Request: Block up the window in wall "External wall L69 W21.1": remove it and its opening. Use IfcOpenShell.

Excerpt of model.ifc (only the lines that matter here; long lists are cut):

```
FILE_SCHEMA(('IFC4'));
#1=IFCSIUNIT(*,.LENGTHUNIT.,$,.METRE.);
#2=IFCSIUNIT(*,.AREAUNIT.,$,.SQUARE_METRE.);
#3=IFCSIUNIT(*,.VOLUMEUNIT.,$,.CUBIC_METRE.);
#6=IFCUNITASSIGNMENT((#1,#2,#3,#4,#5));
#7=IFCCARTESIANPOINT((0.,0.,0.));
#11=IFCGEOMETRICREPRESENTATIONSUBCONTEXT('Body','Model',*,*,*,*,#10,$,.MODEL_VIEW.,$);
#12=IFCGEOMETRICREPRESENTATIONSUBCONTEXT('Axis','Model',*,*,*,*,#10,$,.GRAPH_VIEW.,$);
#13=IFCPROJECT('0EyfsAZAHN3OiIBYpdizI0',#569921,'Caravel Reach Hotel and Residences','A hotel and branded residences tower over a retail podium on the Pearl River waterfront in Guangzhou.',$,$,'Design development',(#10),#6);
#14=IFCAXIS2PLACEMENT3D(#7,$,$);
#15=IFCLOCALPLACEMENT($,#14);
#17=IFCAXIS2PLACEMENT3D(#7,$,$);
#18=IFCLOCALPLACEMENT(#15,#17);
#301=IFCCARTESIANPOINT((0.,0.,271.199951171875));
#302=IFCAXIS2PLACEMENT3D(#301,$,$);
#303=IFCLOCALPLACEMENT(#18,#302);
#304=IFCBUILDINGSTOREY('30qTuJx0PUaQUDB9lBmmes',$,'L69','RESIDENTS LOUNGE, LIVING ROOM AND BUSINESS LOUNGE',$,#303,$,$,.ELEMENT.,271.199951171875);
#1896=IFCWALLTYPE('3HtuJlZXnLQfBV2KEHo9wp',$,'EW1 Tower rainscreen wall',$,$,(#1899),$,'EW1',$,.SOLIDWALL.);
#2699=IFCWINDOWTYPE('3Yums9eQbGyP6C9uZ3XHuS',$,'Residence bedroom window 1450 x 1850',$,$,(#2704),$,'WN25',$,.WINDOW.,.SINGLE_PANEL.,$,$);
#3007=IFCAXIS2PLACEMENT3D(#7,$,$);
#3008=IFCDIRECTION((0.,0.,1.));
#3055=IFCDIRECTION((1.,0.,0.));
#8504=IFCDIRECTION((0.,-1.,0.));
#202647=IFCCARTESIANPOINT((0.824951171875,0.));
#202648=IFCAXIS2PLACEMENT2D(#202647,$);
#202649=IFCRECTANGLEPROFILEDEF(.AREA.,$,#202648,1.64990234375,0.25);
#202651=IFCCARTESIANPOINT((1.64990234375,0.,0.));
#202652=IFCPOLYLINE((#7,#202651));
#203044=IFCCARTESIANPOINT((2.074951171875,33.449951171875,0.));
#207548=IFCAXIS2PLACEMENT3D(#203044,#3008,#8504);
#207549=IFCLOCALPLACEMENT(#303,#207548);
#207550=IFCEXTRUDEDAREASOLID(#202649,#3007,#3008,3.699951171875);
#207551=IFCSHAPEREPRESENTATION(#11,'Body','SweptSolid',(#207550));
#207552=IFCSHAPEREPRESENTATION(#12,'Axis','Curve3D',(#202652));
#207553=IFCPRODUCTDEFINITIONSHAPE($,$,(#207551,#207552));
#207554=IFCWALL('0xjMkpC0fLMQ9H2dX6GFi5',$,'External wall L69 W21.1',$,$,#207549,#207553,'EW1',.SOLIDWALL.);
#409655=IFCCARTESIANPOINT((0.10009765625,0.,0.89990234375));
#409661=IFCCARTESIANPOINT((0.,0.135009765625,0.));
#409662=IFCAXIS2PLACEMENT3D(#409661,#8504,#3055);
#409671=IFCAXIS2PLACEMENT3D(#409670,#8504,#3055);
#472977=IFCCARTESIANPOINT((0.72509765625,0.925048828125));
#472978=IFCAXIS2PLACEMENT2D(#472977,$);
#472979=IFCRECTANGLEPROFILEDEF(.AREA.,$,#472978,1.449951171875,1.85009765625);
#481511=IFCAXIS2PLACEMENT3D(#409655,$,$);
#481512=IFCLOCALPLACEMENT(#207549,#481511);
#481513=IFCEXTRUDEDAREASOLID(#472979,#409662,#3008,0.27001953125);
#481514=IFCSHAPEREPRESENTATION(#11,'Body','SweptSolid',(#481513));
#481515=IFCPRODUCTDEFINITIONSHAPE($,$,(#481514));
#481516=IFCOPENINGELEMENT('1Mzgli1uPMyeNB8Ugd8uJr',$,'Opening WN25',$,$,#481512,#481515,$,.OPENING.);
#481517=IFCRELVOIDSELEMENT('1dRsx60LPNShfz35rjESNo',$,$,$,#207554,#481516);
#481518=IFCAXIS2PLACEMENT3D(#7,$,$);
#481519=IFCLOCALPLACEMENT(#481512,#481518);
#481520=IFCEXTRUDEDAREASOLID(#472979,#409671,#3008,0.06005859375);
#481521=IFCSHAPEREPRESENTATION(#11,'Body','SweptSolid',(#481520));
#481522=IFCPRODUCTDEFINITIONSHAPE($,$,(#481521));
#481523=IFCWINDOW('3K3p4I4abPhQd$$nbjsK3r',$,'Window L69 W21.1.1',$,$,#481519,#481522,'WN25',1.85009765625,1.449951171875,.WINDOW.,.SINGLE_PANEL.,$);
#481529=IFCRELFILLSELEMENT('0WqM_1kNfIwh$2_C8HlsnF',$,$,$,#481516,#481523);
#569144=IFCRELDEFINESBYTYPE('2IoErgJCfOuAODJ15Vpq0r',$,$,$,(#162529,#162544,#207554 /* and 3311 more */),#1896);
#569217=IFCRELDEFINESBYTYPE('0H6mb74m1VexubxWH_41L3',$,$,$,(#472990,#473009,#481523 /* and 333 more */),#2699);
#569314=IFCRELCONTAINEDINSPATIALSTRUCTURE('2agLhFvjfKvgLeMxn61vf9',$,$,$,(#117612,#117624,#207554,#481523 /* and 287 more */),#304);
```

```python
import ifcopenshell
import ifcopenshell.api.feature
import ifcopenshell.api.root
import ifcopenshell.geom
import ifcopenshell.util.shape

model = ifcopenshell.open("model.ifc")
settings = ifcopenshell.geom.settings()


def volume(element):
    """Net volume in cubic metres, openings subtracted."""
    shape = ifcopenshell.geom.create_shape(settings, element)
    return ifcopenshell.util.shape.get_volume(shape.geometry)


window = model.by_guid("3K3p4I4abPhQd$$nbjsK3r")
opening = window.FillsVoids[0].RelatingOpeningElement
wall = opening.VoidsElements[0].RelatingBuildingElement
before = volume(wall)

ifcopenshell.api.root.remove_product(model, product=window)
ifcopenshell.api.feature.remove_feature(model, feature=opening)

after = volume(wall)

print(f"wall volume {before:.3f} -> {after:.3f} m3")

model.write("model_edited.ifc")
```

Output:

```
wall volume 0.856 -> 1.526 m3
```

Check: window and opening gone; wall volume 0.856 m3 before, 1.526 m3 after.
